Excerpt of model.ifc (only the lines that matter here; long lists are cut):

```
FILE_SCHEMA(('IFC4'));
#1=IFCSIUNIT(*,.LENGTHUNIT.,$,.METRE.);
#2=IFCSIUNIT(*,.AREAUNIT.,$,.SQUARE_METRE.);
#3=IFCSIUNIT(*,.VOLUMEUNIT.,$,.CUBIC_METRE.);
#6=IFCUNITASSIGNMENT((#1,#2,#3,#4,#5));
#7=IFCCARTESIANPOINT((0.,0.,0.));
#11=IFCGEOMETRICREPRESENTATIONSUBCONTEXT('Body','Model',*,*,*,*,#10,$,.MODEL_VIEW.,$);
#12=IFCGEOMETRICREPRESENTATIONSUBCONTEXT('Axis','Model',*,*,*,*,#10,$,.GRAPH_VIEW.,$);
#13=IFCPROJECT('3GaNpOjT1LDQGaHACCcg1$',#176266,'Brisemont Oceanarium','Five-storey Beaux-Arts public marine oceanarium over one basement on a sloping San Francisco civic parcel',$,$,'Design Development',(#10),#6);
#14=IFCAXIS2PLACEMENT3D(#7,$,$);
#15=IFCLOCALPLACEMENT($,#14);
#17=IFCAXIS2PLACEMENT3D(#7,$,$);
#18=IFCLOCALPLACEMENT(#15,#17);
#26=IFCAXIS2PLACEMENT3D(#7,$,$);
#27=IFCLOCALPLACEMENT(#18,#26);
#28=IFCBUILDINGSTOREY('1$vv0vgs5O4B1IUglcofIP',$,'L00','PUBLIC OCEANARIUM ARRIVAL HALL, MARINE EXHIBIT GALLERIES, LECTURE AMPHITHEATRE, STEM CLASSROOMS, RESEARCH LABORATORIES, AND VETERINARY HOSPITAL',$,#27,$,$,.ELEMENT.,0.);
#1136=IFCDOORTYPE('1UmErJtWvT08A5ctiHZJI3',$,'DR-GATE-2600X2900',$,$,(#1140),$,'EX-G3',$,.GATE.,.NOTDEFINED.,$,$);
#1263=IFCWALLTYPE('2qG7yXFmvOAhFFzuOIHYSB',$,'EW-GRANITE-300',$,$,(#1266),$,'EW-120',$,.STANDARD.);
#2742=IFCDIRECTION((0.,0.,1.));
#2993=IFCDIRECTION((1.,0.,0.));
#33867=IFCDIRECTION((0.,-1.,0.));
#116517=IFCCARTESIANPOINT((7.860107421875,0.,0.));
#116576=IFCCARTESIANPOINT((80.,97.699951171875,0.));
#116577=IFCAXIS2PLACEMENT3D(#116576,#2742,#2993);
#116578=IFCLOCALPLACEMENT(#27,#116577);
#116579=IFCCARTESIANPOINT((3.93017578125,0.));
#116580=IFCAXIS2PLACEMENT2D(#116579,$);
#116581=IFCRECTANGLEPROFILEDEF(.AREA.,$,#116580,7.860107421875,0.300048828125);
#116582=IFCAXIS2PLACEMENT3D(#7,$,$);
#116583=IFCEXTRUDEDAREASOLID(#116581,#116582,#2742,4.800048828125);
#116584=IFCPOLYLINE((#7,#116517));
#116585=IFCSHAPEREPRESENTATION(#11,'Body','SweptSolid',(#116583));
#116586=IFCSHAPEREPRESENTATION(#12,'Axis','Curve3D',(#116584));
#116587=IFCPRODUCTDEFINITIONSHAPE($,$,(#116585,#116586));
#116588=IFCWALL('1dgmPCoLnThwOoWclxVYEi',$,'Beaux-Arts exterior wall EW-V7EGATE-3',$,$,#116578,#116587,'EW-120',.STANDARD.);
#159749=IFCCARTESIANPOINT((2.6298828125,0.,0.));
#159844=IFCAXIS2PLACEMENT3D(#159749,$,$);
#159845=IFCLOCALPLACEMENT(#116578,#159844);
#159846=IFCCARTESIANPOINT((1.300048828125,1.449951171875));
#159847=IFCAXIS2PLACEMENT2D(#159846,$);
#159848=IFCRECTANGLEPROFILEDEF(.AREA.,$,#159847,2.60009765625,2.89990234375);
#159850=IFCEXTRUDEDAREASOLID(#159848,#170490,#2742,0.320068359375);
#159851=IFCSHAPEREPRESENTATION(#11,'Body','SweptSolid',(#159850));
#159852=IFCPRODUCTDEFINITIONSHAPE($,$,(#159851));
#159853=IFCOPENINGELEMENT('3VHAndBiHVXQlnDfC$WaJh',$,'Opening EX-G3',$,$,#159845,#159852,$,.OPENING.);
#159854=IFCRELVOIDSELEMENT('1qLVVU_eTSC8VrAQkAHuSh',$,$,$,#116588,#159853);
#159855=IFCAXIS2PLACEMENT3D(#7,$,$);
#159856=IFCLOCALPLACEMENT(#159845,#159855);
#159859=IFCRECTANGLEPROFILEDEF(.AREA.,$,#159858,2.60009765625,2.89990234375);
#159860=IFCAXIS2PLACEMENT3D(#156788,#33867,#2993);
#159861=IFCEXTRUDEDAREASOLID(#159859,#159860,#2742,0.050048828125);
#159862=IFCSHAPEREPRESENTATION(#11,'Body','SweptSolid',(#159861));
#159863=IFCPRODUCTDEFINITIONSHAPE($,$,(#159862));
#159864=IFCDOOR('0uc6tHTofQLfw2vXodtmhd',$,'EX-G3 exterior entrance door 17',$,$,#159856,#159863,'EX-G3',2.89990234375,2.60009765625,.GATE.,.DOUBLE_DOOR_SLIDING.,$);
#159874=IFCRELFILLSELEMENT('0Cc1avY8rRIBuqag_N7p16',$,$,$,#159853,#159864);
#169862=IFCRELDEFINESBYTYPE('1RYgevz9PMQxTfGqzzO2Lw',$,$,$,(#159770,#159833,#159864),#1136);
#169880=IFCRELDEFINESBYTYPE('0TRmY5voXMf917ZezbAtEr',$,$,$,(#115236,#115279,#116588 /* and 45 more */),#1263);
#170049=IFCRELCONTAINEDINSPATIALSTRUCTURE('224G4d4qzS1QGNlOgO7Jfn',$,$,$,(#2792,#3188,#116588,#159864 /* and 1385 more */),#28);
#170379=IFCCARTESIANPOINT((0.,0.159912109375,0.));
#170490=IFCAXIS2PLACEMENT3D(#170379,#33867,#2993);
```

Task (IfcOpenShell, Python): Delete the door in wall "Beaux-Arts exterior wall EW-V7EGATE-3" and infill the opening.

```python
import ifcopenshell
import ifcopenshell.api.feature
import ifcopenshell.api.root
import ifcopenshell.geom
import ifcopenshell.util.shape

model = ifcopenshell.open("model.ifc")
settings = ifcopenshell.geom.settings()


def volume(element):
    """Net volume in cubic metres, openings subtracted."""
    shape = ifcopenshell.geom.create_shape(settings, element)
    return ifcopenshell.util.shape.get_volume(shape.geometry)


door = model.by_guid("0uc6tHTofQLfw2vXodtmhd")
opening = door.FillsVoids[0].RelatingOpeningElement
wall = opening.VoidsElements[0].RelatingBuildingElement
before = volume(wall)

ifcopenshell.api.root.remove_product(model, product=door)
ifcopenshell.api.feature.remove_feature(model, feature=opening)

after = volume(wall)

print(f"wall volume {before:.3f} -> {after:.3f} m3")

model.write("model_rev.ifc")
```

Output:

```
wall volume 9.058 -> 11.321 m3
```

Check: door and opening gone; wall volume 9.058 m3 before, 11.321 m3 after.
